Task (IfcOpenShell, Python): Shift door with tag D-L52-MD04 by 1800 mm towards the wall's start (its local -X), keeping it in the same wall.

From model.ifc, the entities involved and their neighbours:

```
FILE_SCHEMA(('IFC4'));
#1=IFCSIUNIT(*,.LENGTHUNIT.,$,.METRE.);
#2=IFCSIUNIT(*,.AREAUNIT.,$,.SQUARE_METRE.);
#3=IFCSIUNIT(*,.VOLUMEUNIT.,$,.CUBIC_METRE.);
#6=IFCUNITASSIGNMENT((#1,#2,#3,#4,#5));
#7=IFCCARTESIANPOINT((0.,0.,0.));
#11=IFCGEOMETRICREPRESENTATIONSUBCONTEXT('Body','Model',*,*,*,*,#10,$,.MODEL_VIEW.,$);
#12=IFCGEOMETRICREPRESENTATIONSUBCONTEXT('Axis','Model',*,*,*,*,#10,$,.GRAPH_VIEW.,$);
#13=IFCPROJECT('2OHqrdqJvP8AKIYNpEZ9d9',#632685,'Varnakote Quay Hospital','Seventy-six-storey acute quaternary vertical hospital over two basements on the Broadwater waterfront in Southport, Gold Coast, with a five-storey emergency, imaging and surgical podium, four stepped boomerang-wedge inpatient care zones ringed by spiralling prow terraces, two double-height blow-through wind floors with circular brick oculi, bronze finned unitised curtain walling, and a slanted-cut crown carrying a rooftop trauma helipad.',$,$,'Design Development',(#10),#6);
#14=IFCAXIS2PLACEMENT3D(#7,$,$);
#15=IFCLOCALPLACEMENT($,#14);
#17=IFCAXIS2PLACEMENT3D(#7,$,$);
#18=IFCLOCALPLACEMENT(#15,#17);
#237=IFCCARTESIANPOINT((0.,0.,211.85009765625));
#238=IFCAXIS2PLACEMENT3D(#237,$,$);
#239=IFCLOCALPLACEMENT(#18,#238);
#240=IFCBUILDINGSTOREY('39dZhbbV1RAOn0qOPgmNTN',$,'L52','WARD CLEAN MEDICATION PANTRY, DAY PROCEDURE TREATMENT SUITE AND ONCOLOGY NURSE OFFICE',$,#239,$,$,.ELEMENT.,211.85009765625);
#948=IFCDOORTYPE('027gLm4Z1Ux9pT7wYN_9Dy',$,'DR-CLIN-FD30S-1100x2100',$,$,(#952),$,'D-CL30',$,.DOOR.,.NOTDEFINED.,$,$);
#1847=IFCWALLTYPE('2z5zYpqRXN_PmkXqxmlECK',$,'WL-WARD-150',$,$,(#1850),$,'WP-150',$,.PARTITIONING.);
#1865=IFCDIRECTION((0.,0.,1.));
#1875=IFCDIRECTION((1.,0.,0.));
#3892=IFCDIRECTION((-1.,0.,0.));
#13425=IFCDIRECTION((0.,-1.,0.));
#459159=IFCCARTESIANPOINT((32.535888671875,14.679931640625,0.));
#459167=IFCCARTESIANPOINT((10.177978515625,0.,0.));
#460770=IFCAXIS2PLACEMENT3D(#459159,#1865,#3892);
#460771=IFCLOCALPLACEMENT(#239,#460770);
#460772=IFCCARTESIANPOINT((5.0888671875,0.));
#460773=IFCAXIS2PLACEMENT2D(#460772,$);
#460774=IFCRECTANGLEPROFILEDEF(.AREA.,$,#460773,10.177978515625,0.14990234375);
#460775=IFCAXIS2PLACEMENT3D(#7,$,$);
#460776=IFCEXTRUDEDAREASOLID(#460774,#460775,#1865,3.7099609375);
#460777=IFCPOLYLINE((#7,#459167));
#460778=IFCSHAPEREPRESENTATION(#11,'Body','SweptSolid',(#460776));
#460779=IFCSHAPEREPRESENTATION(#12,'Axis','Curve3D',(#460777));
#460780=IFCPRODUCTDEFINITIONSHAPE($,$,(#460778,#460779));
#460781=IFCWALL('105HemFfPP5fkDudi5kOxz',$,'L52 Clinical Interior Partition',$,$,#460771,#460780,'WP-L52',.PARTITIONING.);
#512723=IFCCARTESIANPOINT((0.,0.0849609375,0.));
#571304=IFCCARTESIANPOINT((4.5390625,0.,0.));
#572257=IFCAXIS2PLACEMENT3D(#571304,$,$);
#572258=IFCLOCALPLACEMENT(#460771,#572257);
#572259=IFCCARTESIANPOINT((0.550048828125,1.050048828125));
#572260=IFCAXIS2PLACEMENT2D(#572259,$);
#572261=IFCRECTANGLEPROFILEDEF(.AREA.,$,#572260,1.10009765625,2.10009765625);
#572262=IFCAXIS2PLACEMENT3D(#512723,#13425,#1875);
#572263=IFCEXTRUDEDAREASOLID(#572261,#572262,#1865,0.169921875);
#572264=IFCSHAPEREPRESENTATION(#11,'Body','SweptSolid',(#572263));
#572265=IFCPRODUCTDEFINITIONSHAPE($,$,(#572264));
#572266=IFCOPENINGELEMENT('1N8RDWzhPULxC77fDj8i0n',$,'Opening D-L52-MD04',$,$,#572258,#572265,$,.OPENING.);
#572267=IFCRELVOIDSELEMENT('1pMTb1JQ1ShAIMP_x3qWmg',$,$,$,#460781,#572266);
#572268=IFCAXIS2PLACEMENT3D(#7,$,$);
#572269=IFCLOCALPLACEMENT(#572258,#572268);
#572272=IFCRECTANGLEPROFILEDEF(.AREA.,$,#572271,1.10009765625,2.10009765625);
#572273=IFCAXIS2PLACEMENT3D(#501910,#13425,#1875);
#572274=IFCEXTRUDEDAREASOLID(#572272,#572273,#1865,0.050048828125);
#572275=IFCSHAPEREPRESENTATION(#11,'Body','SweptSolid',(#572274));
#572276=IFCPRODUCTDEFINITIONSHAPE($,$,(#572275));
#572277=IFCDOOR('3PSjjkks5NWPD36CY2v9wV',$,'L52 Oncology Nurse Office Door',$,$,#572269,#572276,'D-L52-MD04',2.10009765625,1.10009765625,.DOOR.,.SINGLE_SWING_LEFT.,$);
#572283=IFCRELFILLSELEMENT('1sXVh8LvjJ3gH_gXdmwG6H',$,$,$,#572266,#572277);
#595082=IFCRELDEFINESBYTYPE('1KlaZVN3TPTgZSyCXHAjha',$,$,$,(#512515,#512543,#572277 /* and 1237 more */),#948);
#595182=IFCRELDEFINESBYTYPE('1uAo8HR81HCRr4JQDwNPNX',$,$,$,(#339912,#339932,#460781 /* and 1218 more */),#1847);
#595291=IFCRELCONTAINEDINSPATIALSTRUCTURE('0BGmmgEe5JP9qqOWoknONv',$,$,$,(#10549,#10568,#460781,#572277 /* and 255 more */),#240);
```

```python
import ifcopenshell
import ifcopenshell.api.geometry
import ifcopenshell.util.placement
import ifcopenshell.util.unit

model = ifcopenshell.open("model.ifc")
unit_scale = ifcopenshell.util.unit.calculate_unit_scale(model)

door = model.by_id(572277)
opening = door.FillsVoids[0].RelatingOpeningElement
wall = opening.VoidsElements[0].RelatingBuildingElement

wall_matrix = ifcopenshell.util.placement.get_local_placement(wall.ObjectPlacement)
shift = wall_matrix[:3, 0] * -1.8 / unit_scale
before = ifcopenshell.util.placement.get_local_placement(door.ObjectPlacement)[:3, 3].copy()

# The door is placed relative to its opening, so it follows when the opening moves.
matrix = ifcopenshell.util.placement.get_local_placement(opening.ObjectPlacement)
matrix[:3, 3] += shift
ifcopenshell.api.geometry.edit_object_placement(
    model, product=opening, matrix=matrix, is_si=False, should_transform_children=True
)

after = ifcopenshell.util.placement.get_local_placement(door.ObjectPlacement)[:3, 3]
print("door moved by", (after - before).round(3) + 0.0)

model.write("model_updated.ifc")
```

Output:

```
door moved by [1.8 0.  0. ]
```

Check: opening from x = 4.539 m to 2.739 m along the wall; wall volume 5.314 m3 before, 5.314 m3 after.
